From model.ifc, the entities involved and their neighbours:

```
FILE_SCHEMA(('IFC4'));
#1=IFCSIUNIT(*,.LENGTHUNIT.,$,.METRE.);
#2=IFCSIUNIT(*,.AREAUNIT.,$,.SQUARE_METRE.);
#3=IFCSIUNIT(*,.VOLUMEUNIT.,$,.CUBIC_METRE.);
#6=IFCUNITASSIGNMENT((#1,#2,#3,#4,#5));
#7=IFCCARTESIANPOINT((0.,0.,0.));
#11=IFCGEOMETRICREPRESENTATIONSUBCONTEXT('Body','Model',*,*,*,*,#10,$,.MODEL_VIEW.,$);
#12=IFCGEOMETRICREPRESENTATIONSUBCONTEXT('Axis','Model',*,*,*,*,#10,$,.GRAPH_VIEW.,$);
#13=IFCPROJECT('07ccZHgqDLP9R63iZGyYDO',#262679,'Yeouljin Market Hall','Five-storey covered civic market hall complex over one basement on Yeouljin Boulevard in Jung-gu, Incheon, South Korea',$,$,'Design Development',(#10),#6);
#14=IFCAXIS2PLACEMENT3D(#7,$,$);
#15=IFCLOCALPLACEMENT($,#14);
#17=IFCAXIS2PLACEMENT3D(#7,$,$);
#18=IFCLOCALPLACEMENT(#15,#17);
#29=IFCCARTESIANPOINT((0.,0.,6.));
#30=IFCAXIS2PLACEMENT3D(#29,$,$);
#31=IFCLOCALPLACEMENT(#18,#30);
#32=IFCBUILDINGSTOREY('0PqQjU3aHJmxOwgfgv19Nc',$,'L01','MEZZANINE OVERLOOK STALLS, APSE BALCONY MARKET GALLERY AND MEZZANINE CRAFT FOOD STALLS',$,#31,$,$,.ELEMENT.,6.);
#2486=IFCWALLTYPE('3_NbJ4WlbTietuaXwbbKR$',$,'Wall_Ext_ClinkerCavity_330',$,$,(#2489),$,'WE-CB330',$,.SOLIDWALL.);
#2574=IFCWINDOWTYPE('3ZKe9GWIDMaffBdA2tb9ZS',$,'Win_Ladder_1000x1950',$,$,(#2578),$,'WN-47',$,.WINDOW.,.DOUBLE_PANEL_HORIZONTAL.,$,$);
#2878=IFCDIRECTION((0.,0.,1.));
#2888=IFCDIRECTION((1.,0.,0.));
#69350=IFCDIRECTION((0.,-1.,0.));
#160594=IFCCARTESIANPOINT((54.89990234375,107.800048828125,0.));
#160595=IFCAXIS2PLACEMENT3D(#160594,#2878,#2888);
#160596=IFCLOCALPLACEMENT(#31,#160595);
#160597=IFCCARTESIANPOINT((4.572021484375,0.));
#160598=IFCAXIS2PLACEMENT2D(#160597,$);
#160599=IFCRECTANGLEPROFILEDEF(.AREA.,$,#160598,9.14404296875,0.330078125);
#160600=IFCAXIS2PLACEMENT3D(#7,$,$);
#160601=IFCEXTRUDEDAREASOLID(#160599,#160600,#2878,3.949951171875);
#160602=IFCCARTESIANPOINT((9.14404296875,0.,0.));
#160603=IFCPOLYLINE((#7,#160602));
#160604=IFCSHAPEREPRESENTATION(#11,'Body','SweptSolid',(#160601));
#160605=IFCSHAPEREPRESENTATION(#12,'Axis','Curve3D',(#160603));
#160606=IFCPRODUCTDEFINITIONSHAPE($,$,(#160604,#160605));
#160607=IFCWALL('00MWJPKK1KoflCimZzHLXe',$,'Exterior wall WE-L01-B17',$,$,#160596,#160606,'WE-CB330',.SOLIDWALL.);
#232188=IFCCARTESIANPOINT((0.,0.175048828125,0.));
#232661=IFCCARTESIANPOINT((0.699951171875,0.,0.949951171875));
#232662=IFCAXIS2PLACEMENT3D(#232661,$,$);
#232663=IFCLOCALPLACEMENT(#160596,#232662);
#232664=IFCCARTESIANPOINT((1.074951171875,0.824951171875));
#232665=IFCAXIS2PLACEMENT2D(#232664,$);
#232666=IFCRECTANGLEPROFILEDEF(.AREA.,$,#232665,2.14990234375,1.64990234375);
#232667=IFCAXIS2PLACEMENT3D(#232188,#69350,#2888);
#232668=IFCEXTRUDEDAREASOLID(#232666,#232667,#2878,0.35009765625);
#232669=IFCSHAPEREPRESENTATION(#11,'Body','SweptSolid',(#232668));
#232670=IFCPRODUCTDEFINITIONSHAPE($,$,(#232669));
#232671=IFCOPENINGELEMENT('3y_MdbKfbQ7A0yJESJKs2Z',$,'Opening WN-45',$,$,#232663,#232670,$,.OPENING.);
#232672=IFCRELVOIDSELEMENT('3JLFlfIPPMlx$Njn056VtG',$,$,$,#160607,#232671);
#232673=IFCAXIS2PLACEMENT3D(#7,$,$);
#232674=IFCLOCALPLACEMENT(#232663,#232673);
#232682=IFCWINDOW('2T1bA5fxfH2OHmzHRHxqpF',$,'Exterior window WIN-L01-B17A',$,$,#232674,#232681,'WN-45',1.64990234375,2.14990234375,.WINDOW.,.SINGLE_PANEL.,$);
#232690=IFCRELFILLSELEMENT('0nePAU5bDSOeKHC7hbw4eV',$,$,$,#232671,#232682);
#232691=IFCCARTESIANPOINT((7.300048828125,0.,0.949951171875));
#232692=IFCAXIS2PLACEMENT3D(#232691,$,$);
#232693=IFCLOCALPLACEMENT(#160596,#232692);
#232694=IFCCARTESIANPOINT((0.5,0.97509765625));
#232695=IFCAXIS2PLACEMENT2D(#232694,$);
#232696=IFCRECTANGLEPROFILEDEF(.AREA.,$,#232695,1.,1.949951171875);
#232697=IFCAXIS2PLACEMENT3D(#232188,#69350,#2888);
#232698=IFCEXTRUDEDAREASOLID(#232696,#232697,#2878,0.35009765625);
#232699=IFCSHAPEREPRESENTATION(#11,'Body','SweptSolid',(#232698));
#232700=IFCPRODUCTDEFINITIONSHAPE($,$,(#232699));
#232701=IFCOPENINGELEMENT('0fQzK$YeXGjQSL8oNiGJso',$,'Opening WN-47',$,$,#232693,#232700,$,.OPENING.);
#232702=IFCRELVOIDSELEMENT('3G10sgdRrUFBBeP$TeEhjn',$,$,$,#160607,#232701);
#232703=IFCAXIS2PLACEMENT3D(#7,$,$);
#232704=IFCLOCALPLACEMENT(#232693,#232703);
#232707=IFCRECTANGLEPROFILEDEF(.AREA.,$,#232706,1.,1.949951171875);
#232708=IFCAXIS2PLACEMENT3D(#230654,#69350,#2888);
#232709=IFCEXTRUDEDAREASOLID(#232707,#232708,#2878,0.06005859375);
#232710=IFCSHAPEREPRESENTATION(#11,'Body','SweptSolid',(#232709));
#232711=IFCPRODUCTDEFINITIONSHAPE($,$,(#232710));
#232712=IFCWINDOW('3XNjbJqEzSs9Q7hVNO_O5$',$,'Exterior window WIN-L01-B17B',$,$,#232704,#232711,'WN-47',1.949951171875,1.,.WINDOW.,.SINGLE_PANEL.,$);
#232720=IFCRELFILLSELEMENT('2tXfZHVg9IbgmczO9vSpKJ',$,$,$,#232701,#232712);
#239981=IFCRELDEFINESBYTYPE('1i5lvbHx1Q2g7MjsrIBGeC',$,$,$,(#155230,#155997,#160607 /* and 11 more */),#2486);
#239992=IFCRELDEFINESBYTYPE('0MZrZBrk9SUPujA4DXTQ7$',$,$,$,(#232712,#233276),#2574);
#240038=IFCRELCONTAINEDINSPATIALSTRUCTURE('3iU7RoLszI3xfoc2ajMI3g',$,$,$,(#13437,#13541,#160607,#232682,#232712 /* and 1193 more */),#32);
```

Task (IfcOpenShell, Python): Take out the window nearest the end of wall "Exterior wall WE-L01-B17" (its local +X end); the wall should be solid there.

```python
import ifcopenshell
import ifcopenshell.api.feature
import ifcopenshell.api.root
import ifcopenshell.geom
import ifcopenshell.util.shape

model = ifcopenshell.open("model.ifc")
settings = ifcopenshell.geom.settings()


def volume(element):
    """Net volume in cubic metres, openings subtracted."""
    shape = ifcopenshell.geom.create_shape(settings, element)
    return ifcopenshell.util.shape.get_volume(shape.geometry)


window = model.by_id(232712)
opening = window.FillsVoids[0].RelatingOpeningElement
wall = opening.VoidsElements[0].RelatingBuildingElement
before = volume(wall)

ifcopenshell.api.root.remove_product(model, product=window)
ifcopenshell.api.feature.remove_feature(model, feature=opening)

after = volume(wall)

print(f"wall volume {before:.3f} -> {after:.3f} m3")

model.write("model-out.ifc")
```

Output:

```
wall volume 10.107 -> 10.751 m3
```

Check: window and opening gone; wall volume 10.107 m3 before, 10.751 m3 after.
